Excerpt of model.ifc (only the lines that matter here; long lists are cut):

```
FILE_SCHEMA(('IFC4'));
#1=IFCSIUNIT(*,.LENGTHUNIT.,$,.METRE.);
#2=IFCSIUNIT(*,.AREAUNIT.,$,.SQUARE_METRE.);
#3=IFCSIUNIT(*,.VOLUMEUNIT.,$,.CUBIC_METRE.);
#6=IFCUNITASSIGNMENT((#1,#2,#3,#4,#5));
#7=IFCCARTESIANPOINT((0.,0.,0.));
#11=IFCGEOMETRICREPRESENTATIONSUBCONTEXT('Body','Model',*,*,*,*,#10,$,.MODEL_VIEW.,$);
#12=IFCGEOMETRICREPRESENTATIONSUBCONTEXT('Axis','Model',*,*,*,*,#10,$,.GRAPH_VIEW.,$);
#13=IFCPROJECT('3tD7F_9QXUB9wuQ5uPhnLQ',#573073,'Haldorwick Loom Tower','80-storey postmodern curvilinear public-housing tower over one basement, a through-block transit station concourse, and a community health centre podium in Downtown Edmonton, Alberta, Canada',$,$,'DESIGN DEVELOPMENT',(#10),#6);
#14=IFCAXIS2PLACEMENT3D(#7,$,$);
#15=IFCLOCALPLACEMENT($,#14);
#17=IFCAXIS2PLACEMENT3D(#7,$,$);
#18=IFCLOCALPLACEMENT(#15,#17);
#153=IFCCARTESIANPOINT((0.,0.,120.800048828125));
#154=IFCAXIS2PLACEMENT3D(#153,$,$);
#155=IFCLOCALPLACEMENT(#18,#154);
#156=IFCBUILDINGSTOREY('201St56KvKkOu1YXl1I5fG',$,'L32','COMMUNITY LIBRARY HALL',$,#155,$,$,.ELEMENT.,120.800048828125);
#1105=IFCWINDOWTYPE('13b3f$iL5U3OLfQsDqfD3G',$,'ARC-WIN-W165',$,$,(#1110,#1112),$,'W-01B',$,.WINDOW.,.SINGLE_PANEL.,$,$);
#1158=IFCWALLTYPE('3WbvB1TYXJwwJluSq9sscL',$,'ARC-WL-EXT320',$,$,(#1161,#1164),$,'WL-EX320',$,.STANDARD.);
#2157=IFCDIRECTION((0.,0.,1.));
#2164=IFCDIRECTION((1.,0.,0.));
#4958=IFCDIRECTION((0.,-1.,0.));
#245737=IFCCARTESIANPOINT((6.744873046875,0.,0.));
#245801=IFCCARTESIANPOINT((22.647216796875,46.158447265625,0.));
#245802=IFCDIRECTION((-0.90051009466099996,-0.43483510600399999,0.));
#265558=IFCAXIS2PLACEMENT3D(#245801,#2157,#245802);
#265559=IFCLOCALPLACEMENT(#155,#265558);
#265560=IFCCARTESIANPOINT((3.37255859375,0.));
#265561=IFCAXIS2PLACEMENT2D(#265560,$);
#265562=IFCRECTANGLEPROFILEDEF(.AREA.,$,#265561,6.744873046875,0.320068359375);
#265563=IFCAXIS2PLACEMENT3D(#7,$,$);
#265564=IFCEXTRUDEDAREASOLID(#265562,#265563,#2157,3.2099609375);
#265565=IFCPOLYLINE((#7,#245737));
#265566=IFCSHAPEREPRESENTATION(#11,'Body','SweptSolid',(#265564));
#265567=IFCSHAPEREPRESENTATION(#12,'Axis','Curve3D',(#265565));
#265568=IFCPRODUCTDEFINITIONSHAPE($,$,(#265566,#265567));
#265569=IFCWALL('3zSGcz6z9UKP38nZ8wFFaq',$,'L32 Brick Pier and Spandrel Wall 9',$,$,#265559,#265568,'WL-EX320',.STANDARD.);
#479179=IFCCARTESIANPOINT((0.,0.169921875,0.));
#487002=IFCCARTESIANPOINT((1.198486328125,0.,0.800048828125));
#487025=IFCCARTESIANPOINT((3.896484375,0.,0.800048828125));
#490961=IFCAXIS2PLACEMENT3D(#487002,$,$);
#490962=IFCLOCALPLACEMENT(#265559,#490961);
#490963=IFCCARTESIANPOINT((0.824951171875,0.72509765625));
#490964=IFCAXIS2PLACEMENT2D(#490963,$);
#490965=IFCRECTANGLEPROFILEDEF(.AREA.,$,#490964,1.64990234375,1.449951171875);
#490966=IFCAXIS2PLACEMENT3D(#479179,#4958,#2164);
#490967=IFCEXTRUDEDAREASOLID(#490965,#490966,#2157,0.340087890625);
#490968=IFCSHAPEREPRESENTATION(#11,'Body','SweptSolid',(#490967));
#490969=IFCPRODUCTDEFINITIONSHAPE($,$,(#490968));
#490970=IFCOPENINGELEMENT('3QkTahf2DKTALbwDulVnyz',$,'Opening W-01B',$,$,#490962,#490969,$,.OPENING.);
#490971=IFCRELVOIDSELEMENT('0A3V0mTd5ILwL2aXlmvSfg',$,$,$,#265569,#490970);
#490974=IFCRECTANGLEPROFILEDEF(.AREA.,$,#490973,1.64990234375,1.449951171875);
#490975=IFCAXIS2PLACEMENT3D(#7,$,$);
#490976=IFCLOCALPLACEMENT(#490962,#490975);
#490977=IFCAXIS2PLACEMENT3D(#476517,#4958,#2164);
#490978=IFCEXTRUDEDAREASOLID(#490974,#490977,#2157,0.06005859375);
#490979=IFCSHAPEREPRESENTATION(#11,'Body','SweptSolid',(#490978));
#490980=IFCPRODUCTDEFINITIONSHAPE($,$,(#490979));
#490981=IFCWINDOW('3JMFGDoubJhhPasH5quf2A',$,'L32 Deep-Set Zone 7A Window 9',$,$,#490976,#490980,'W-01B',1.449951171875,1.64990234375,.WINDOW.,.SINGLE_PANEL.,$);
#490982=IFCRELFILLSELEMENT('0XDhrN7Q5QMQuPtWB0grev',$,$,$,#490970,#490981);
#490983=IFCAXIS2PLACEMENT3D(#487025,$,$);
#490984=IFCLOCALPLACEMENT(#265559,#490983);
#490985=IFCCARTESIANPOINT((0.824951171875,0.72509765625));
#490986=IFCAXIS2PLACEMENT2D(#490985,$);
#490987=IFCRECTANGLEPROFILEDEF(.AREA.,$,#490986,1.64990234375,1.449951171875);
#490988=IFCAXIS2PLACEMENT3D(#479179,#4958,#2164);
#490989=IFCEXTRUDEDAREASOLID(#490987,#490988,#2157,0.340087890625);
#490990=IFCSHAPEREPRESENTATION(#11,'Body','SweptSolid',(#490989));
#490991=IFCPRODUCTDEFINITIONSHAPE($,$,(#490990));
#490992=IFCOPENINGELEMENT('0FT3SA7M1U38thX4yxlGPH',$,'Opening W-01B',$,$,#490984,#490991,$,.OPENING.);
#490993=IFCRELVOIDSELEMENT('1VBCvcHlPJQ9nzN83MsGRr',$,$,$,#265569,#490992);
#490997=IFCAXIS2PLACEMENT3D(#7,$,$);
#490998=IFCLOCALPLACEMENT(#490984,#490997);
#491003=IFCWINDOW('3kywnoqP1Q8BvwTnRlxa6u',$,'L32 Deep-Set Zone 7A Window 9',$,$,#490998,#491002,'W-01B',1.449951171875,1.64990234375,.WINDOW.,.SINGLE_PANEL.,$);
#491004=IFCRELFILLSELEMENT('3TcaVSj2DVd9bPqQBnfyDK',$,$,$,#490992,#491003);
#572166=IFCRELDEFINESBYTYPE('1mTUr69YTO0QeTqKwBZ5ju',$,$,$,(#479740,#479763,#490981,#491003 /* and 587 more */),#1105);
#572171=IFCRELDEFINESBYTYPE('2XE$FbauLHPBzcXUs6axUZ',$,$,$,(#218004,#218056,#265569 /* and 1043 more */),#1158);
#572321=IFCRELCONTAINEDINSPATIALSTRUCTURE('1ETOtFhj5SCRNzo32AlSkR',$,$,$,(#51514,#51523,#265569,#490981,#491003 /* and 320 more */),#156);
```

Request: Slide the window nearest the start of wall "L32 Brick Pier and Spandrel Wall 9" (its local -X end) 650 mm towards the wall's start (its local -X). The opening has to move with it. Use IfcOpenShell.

```python
import ifcopenshell
import ifcopenshell.api.geometry
import ifcopenshell.util.placement
import ifcopenshell.util.unit

model = ifcopenshell.open("model.ifc")
unit_scale = ifcopenshell.util.unit.calculate_unit_scale(model)

window = model.by_guid("3JMFGDoubJhhPasH5quf2A")
opening = window.FillsVoids[0].RelatingOpeningElement
wall = opening.VoidsElements[0].RelatingBuildingElement

wall_matrix = ifcopenshell.util.placement.get_local_placement(wall.ObjectPlacement)
shift = wall_matrix[:3, 0] * -0.65 / unit_scale
before = ifcopenshell.util.placement.get_local_placement(window.ObjectPlacement)[:3, 3].copy()

# The window is placed relative to its opening, so it follows when the opening moves.
matrix = ifcopenshell.util.placement.get_local_placement(opening.ObjectPlacement)
matrix[:3, 3] += shift
ifcopenshell.api.geometry.edit_object_placement(
    model, product=opening, matrix=matrix, is_si=False, should_transform_children=True
)

after = ifcopenshell.util.placement.get_local_placement(window.ObjectPlacement)[:3, 3]
print("window moved by", (after - before).round(3) + 0.0)

model.write("model-out.ifc")
```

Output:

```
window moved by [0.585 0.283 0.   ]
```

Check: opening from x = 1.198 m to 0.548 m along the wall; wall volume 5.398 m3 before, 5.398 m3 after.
